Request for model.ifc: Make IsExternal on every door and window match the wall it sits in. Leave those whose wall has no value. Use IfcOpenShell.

First a look at what the model holds.

```python
import ifcopenshell
import ifcopenshell.util.element

model = ifcopenshell.open("model.ifc")
print(model.schema)
seen = {}
for e in model.by_type("IfcDoor") + model.by_type("IfcWindow"):
    if not e.FillsVoids:
        continue
    host = e.FillsVoids[0].RelatingOpeningElement.VoidsElements[0].RelatingBuildingElement
    own = ifcopenshell.util.element.get_pset(e, f"Pset_{e.is_a()[3:].removesuffix('StandardCase')}Common", "IsExternal")
    wall = ifcopenshell.util.element.get_pset(host, "Pset_WallCommon", "IsExternal")
    seen[e.is_a(), own, wall] = seen.get((e.is_a(), own, wall), 0) + 1
for (cls, own, wall), count in sorted(seen.items(), key=str):
    print(count, cls, "IsExternal:", own, "| host wall:", wall)
```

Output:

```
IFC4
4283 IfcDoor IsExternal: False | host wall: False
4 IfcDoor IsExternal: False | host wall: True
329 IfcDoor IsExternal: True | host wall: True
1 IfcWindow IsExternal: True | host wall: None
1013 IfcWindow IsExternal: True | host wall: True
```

```python
import ifcopenshell
import ifcopenshell.api.pset
import ifcopenshell.util.element

model = ifcopenshell.open("model.ifc")

count = 0
for ifc_class, pset_name in (("IfcDoor", "Pset_DoorCommon"), ("IfcWindow", "Pset_WindowCommon")):
    for e in model.by_type(ifc_class):
        if not e.FillsVoids:
            continue
        host = e.FillsVoids[0].RelatingOpeningElement.VoidsElements[0].RelatingBuildingElement
        external = ifcopenshell.util.element.get_pset(host, "Pset_WallCommon", "IsExternal")
        if external is None or ifcopenshell.util.element.get_pset(e, pset_name, "IsExternal") == external:
            continue
        found = ifcopenshell.util.element.get_pset(e, pset_name, should_inherit=False)
        if found:
            pset = model.by_id(found["id"])
            if len(ifcopenshell.util.element.get_elements_by_pset(pset)) > 1:
                pset = ifcopenshell.api.pset.unshare_pset(model, products=[e], pset=pset)[0]
        else:
            pset = ifcopenshell.api.pset.add_pset(model, product=e, name=pset_name)
        ifcopenshell.api.pset.edit_pset(model, pset=pset, properties={"IsExternal": external})
        count += 1

print(count, "updated")

model.write("model_edited.ifc")
```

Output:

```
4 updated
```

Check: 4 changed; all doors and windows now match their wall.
